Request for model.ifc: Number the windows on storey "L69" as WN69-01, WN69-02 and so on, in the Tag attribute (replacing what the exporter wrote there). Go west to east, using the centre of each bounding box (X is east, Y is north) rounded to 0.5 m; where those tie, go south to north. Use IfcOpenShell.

First a look at what the model holds.

```python
import ifcopenshell
import ifcopenshell.util.element
import ifcopenshell.util.placement

model = ifcopenshell.open("model.ifc")
print(model.schema)
storey = next(s for s in model.by_type("IfcBuildingStorey") if s.Name == "L69")
windows = [e for e in ifcopenshell.util.element.get_decomposition(storey) if e.is_a("IfcWindow")]
for e in sorted(windows, key=lambda e: e.id()):
    origin = ifcopenshell.util.placement.get_local_placement(e.ObjectPlacement)[:3, 3]
    print(e.id(), e.Tag, e.Name, origin.round(2) + 0.0, sep=" | ")
```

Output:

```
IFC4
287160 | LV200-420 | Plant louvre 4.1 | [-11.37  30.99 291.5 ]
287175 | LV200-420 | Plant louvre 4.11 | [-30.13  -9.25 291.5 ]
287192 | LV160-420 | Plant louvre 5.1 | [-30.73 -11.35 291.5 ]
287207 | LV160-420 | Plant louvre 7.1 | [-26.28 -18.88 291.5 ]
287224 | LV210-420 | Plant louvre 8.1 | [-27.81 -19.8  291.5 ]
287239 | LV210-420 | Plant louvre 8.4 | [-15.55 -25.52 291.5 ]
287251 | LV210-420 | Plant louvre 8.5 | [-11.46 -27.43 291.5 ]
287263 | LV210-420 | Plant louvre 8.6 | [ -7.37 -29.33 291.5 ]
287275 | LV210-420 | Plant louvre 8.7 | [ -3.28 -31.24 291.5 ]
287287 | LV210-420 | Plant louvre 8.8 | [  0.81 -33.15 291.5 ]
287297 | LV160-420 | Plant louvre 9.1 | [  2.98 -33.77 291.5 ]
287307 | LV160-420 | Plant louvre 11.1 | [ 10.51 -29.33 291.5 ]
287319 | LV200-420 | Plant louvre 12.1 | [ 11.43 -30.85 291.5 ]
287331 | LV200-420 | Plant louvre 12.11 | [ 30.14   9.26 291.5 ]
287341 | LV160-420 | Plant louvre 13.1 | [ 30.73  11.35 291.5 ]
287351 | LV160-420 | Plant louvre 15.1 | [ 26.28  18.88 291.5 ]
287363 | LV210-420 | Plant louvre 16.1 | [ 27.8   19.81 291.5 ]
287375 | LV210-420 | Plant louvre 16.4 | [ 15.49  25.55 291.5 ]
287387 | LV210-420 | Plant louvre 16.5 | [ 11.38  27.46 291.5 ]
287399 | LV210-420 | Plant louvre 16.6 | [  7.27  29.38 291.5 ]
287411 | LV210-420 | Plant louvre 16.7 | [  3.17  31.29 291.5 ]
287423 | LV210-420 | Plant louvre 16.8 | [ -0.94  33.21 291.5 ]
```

```python
import ifcopenshell
import ifcopenshell.geom
import ifcopenshell.util.element
import ifcopenshell.util.shape

model = ifcopenshell.open("model.ifc")
settings = ifcopenshell.geom.settings()
settings.set("use-world-coords", True)


def centre(element):
    shape = ifcopenshell.geom.create_shape(settings, element)
    return ifcopenshell.util.shape.get_bbox_centroid(shape.geometry)


storey = next(s for s in model.by_type("IfcBuildingStorey") if s.Name == "L69")
windows = [e for e in ifcopenshell.util.element.get_decomposition(storey) if e.is_a("IfcWindow")]

# Insertion points can sit at a corner or the storey origin, so sort by the geometry (in metres).
centres = {e: centre(e) for e in windows}
windows.sort(key=lambda e: (round(centres[e][0] / 0.5), centres[e][1]))

for i, e in enumerate(windows, start=1):
    number = f"WN69-{i:02d}"
    e.Tag = number
    print(e.id(), number)

model.write("model-out.ifc")
```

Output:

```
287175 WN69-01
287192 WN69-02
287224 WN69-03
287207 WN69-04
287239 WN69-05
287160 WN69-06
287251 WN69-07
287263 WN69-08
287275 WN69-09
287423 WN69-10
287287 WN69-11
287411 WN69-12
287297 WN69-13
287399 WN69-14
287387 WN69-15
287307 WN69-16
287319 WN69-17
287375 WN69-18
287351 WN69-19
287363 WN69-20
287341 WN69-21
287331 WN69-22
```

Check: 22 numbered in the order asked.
